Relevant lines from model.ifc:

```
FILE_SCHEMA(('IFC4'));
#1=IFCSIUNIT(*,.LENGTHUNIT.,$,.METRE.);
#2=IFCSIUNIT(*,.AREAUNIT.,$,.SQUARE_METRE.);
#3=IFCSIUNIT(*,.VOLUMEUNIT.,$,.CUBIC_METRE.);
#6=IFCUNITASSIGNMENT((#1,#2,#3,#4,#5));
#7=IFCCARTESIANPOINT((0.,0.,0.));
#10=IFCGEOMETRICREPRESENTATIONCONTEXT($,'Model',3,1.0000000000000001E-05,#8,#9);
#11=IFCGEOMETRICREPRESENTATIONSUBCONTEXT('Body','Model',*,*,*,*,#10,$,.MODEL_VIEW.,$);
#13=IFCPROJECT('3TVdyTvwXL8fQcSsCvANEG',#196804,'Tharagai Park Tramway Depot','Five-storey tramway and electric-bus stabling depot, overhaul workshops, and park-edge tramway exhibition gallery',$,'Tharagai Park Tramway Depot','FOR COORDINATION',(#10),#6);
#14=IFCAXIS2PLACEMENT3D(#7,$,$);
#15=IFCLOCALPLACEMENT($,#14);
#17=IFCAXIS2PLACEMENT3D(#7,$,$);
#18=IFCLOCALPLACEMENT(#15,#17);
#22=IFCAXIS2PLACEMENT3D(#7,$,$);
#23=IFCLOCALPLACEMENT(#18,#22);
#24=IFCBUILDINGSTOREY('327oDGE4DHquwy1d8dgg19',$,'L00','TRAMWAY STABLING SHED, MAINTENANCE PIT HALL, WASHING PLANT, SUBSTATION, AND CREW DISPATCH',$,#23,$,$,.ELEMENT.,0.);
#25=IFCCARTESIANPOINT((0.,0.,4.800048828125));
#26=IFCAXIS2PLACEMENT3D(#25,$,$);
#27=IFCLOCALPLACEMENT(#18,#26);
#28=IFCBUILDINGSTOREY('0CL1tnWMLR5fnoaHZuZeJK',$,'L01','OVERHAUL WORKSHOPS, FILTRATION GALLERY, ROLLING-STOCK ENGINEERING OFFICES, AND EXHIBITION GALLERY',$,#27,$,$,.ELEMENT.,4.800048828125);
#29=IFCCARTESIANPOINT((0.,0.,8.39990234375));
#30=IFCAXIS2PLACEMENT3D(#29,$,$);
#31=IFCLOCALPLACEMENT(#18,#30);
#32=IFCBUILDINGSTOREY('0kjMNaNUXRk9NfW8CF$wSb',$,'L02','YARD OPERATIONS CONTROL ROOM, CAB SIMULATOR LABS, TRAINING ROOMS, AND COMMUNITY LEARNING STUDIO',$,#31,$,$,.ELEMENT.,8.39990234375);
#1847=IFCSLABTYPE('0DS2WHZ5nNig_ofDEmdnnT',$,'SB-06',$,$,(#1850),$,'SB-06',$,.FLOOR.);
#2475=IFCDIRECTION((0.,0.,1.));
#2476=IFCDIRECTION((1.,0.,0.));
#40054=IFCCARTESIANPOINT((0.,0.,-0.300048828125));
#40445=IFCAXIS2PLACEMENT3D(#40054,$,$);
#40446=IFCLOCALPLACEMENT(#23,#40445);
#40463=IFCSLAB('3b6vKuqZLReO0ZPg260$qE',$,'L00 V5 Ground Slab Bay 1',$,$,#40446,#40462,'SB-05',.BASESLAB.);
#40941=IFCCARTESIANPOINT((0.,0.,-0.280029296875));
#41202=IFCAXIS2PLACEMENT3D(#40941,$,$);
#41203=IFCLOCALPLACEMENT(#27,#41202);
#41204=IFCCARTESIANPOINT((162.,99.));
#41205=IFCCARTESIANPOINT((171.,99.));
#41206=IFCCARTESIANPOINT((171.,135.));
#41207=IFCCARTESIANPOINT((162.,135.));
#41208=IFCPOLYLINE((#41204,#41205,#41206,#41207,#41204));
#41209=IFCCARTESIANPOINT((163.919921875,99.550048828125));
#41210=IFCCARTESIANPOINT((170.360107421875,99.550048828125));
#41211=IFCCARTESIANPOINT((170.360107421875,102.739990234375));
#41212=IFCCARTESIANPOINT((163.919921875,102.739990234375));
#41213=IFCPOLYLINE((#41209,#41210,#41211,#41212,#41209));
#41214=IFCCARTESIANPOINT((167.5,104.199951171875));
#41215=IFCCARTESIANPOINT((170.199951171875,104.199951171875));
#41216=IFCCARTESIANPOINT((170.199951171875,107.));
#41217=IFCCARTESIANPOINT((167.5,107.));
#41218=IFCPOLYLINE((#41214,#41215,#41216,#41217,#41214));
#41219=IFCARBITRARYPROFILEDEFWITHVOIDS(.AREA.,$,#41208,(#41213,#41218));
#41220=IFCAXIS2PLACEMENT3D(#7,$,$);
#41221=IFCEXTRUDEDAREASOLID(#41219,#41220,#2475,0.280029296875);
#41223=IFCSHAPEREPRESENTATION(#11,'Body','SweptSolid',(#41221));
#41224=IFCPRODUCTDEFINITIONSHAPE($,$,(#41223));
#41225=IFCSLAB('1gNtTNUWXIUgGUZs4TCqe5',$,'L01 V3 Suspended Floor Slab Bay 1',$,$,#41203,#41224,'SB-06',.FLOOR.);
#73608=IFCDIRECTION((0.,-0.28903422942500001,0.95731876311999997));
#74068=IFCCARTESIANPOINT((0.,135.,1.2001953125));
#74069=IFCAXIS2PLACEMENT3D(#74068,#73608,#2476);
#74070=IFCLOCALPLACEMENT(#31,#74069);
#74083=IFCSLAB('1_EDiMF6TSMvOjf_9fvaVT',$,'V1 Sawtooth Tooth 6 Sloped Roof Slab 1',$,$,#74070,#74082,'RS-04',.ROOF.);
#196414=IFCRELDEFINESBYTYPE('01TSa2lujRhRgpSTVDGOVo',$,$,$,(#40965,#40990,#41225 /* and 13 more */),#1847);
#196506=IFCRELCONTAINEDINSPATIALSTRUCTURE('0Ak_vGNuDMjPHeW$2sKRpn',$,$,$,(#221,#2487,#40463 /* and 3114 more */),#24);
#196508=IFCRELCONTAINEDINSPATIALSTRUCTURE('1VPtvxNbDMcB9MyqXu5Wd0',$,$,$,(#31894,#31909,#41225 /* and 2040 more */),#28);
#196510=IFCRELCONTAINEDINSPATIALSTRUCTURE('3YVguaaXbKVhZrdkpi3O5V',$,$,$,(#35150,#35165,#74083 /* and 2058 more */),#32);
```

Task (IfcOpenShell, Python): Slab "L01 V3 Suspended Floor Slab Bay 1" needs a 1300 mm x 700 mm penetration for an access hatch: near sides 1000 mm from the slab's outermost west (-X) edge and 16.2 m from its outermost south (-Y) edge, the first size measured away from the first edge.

```python
import numpy as np
import ifcopenshell
import ifcopenshell.api.feature
import ifcopenshell.api.geometry
import ifcopenshell.api.root
import ifcopenshell.geom
import ifcopenshell.util.placement
import ifcopenshell.util.representation
import ifcopenshell.util.shape
import ifcopenshell.util.unit

model = ifcopenshell.open("model.ifc")
unit_scale = ifcopenshell.util.unit.calculate_unit_scale(model)
settings = ifcopenshell.geom.settings()


def volume(element):
    """Net volume in cubic metres, openings subtracted."""
    shape = ifcopenshell.geom.create_shape(settings, element)
    return ifcopenshell.util.shape.get_volume(shape.geometry)


slab = model.by_guid("1gNtTNUWXIUgGUZs4TCqe5")
before = volume(slab)

# Extent in the slab's own axes, in metres. The edges named are its -X and -Y sides.
slab_shape = ifcopenshell.geom.create_shape(settings, slab)
vertices = ifcopenshell.util.shape.get_vertices(slab_shape.geometry)
x_min, y_min, bottom = vertices.min(axis=0)
top = vertices[:, 2].max()

opening = ifcopenshell.api.root.create_entity(model, ifc_class="IfcOpeningElement", name="Access hatch opening", predefined_type="OPENING")
context = ifcopenshell.util.representation.get_context(model, "Model", "Body", "MODEL_VIEW")
width, depth = 1.3, 0.7
outline = [(0.0, 0.0), (width, 0.0), (width, depth), (0.0, depth), (0.0, 0.0)]
# Overshoot both faces by 50 mm so the cut is clean.
shape = ifcopenshell.api.geometry.add_slab_representation(
    model, context=context, depth=top - bottom + 0.1, polyline=outline
)
ifcopenshell.api.geometry.assign_representation(model, product=opening, representation=shape)

matrix = ifcopenshell.util.placement.get_local_placement(slab.ObjectPlacement)
matrix[:, 3] = matrix @ np.append(np.array([x_min + 1, y_min + 16.2, bottom - 0.05]) / unit_scale, 1.0)
ifcopenshell.api.geometry.edit_object_placement(model, product=opening, matrix=matrix, is_si=False)
ifcopenshell.api.feature.add_feature(model, feature=opening, element=slab)

after = volume(slab)

print(f"slab volume {before:.3f} -> {after:.3f} m3")

model.write("model-out.ifc")
```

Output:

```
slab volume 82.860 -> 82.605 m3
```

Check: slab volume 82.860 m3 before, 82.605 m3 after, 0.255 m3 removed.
